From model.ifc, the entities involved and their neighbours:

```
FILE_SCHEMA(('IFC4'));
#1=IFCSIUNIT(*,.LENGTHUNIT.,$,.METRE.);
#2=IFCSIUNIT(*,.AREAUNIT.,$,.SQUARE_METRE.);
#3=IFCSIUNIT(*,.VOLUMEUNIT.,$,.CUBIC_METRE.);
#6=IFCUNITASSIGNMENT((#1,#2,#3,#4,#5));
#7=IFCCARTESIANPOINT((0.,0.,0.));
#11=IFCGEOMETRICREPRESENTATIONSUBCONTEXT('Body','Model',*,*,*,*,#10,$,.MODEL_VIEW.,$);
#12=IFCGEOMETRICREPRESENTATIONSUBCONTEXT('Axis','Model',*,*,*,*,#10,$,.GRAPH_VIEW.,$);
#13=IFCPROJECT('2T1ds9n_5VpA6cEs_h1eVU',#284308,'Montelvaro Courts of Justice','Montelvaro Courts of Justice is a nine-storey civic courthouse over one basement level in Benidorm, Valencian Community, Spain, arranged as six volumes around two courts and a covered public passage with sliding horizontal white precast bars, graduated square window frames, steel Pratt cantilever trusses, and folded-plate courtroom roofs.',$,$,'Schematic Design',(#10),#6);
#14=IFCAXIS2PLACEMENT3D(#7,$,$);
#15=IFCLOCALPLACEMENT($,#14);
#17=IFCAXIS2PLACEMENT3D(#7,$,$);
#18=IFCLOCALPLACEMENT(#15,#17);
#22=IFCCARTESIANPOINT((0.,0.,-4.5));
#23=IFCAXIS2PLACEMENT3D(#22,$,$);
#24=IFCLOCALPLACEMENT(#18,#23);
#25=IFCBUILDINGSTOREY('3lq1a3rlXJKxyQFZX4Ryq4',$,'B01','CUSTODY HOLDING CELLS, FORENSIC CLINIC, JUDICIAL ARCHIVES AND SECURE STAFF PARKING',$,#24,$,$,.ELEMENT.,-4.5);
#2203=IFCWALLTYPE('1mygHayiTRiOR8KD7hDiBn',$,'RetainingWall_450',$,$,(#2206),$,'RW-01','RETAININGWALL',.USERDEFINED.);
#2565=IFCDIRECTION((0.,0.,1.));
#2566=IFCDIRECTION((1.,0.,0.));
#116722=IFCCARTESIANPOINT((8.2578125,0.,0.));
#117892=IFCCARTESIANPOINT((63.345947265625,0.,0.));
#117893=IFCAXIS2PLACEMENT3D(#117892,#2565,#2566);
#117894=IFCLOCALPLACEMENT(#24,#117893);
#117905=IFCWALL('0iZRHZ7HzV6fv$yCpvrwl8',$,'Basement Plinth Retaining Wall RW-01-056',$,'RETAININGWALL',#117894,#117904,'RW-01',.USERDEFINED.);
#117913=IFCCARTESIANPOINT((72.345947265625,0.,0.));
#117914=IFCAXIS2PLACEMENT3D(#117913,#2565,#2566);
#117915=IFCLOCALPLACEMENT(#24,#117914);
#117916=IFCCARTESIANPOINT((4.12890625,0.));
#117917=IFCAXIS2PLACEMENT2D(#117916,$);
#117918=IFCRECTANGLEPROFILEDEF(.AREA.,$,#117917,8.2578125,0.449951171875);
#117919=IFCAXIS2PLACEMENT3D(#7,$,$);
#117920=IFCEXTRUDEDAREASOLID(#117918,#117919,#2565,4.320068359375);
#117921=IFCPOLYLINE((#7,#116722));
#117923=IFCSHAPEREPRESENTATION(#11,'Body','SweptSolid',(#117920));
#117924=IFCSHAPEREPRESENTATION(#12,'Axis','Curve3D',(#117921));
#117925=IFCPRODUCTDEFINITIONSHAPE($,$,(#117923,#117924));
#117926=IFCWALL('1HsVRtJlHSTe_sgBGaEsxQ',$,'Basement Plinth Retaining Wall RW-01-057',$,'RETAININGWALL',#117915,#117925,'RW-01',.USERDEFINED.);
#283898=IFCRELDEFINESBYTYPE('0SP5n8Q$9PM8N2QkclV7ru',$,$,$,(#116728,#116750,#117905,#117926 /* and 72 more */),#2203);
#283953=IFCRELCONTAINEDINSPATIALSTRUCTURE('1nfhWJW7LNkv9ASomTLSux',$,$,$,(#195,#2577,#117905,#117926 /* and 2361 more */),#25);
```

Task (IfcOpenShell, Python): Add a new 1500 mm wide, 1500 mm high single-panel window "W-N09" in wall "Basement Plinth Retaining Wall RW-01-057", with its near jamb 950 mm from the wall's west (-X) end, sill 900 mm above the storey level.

```python
import numpy as np
import ifcopenshell
import ifcopenshell.api.feature
import ifcopenshell.api.geometry
import ifcopenshell.api.root
import ifcopenshell.api.spatial
import ifcopenshell.geom
import ifcopenshell.util.element
import ifcopenshell.util.placement
import ifcopenshell.util.representation
import ifcopenshell.util.shape
import ifcopenshell.util.unit

model = ifcopenshell.open("model.ifc")
unit_scale = ifcopenshell.util.unit.calculate_unit_scale(model)
settings = ifcopenshell.geom.settings()


def volume(element):
    """Net volume in cubic metres, openings subtracted."""
    shape = ifcopenshell.geom.create_shape(settings, element)
    return ifcopenshell.util.shape.get_volume(shape.geometry)


wall = model.by_guid("1HsVRtJlHSTe_sgBGaEsxQ")
storey = ifcopenshell.util.element.get_container(wall, ifc_class="IfcBuildingStorey")
context = ifcopenshell.util.representation.get_context(model, "Model", "Body", "MODEL_VIEW")
before = volume(wall)

width, height, from_end, sill = 1.5, 1.5, 0.95, 0.9  # metres

# The wall runs along its own X axis, and the end named is its -X end.
wall_shape = ifcopenshell.geom.create_shape(settings, wall)
x, y, z = ifcopenshell.util.shape.get_vertices(wall_shape.geometry).T
start = x.min() + from_end
face, thickness = float(y.min()), float(y.max() - y.min())
wall_matrix = ifcopenshell.util.placement.get_local_placement(wall.ObjectPlacement)
level = ifcopenshell.util.placement.get_local_placement(storey.ObjectPlacement)[2, 3]


def in_wall(x, y):
    """Placement at x, y metres in the wall's axes, at sill height."""
    matrix = wall_matrix.copy()
    matrix[:, 3] = wall_matrix @ np.array([x / unit_scale, y / unit_scale, 0.0, 1.0])
    matrix[2, 3] = level + sill / unit_scale
    return matrix


# Opening: a box that overshoots both wall faces by 50 mm.
opening = ifcopenshell.api.root.create_entity(model, ifc_class="IfcOpeningElement", predefined_type="OPENING")
box = ifcopenshell.api.geometry.add_wall_representation(
    model, context=context, length=width, height=height, thickness=thickness + 0.1
)
ifcopenshell.api.geometry.assign_representation(model, product=opening, representation=box)
ifcopenshell.api.geometry.edit_object_placement(model, product=opening, matrix=in_wall(start, face - 0.05), is_si=False)
ifcopenshell.api.feature.add_feature(model, feature=opening, element=wall)

window = ifcopenshell.api.root.create_entity(model, ifc_class="IfcWindow", name="W-N09", predefined_type="WINDOW")
window.OverallWidth, window.OverallHeight = width / unit_scale, height / unit_scale
window.PartitioningType = "SINGLE_PANEL"
body = ifcopenshell.api.geometry.add_window_representation(
    model,
    context=context,
    overall_width=window.OverallWidth,
    overall_height=window.OverallHeight,
    partition_type="SINGLE_PANEL",
)
ifcopenshell.api.geometry.assign_representation(model, product=window, representation=body)
ifcopenshell.api.spatial.assign_container(model, products=[window], relating_structure=storey)
ifcopenshell.api.feature.add_filling(model, opening=opening, element=window)

# Centre the window in the wall's thickness.
ifcopenshell.api.geometry.edit_object_placement(model, product=window, matrix=in_wall(start, face), is_si=False)
window_shape = ifcopenshell.geom.create_shape(settings, window)
depth = ifcopenshell.util.shape.get_vertices(window_shape.geometry)[:, 1]
offset = face + thickness / 2 - (depth.min() + depth.max()) / 2
ifcopenshell.api.geometry.edit_object_placement(model, product=window, matrix=in_wall(start, offset), is_si=False)

after = volume(wall)

print(f"wall volume {before:.3f} -> {after:.3f} m3")

model.write("model-out.ifc")
```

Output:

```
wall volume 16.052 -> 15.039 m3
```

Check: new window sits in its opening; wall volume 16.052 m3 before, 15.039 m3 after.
